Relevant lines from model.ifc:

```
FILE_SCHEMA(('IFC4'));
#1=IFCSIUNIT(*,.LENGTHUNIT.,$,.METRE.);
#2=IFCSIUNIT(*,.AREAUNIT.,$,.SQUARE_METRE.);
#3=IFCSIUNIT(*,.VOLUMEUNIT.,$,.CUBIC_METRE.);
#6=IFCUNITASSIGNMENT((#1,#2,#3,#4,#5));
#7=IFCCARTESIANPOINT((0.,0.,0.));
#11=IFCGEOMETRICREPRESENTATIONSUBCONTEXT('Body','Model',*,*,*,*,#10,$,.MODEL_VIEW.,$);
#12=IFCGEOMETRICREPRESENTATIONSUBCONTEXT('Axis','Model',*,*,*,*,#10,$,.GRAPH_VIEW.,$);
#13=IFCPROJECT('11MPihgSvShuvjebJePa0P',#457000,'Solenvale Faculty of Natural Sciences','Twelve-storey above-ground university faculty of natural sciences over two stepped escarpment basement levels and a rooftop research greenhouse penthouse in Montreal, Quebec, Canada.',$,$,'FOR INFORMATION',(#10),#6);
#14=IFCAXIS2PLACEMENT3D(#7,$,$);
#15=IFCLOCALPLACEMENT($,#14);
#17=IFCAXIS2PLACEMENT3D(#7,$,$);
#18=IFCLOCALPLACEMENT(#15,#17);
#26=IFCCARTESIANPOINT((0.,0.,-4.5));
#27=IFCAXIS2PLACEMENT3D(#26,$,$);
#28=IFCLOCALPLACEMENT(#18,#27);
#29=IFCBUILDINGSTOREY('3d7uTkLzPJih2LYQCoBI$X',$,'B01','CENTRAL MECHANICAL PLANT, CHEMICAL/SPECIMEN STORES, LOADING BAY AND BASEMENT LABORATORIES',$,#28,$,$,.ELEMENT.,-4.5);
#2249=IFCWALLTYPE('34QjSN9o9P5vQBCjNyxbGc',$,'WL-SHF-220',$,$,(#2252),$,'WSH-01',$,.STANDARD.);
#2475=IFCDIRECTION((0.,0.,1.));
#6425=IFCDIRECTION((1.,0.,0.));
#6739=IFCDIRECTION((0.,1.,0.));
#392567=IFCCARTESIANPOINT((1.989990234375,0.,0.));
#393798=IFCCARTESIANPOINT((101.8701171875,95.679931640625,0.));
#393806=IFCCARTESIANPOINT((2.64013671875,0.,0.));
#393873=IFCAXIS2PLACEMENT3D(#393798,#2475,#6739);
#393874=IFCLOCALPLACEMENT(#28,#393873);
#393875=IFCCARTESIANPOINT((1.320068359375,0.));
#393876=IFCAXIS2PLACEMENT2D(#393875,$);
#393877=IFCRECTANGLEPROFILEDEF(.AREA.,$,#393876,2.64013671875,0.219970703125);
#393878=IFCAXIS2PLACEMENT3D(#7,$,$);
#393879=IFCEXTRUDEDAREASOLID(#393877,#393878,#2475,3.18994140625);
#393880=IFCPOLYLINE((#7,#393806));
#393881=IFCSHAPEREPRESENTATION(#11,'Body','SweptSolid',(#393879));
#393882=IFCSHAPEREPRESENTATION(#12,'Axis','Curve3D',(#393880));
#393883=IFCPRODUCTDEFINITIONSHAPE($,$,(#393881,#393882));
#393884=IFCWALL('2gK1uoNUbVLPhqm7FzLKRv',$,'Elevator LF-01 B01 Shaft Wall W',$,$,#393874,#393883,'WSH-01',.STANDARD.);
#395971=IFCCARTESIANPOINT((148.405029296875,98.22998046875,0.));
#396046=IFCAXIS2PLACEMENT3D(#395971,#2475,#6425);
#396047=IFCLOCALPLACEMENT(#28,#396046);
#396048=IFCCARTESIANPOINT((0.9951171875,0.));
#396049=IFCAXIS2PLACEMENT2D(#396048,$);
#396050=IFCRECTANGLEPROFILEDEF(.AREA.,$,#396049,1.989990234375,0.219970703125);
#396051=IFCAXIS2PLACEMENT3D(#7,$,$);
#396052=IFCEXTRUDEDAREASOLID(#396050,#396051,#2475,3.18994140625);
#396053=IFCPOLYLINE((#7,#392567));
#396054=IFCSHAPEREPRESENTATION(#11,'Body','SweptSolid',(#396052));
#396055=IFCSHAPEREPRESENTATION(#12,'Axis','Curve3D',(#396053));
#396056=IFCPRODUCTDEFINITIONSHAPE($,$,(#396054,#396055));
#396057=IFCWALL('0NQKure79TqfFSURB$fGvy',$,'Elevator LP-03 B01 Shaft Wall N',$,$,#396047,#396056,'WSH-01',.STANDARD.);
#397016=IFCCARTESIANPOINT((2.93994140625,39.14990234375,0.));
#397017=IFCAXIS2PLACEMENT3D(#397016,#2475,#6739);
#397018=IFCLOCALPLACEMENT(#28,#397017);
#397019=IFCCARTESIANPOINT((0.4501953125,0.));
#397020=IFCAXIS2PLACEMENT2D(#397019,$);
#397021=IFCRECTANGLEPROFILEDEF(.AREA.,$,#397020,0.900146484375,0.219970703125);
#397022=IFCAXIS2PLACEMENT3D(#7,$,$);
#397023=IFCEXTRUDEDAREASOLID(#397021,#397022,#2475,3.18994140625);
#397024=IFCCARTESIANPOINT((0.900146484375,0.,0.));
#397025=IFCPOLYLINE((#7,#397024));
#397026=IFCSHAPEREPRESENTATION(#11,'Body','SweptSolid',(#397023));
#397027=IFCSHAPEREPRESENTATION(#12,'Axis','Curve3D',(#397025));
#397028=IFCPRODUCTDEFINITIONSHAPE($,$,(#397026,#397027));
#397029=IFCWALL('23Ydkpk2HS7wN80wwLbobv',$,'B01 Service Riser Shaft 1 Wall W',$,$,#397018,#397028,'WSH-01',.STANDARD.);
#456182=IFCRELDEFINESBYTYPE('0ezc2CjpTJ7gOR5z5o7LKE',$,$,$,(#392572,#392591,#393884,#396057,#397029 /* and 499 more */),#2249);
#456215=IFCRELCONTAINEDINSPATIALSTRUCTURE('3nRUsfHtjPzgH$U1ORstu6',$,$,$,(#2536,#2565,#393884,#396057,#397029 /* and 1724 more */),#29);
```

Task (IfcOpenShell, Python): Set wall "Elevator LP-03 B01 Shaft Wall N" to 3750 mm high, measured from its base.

```python
import ifcopenshell
import ifcopenshell.geom
import ifcopenshell.util.representation
import ifcopenshell.util.shape
import ifcopenshell.util.unit

model = ifcopenshell.open("model.ifc")
unit_scale = ifcopenshell.util.unit.calculate_unit_scale(model)
settings = ifcopenshell.geom.settings()


def volume(element):
    """Net volume in cubic metres, openings subtracted."""
    shape = ifcopenshell.geom.create_shape(settings, element)
    return ifcopenshell.util.shape.get_volume(shape.geometry)


wall = model.by_id(396057)
before = volume(wall)

body = ifcopenshell.util.representation.get_representation(wall, "Model", "Body")
solid = body.Items[0]
old_height = solid.Depth
solid.Depth = 3.75 / unit_scale
after = volume(wall)

print(f"height {old_height:g} -> {solid.Depth:g}, volume {before:.3f} -> {after:.3f} m3")

model.write("model_rev.ifc")
```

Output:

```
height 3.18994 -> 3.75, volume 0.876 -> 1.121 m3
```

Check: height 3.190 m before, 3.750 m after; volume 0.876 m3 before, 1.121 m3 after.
